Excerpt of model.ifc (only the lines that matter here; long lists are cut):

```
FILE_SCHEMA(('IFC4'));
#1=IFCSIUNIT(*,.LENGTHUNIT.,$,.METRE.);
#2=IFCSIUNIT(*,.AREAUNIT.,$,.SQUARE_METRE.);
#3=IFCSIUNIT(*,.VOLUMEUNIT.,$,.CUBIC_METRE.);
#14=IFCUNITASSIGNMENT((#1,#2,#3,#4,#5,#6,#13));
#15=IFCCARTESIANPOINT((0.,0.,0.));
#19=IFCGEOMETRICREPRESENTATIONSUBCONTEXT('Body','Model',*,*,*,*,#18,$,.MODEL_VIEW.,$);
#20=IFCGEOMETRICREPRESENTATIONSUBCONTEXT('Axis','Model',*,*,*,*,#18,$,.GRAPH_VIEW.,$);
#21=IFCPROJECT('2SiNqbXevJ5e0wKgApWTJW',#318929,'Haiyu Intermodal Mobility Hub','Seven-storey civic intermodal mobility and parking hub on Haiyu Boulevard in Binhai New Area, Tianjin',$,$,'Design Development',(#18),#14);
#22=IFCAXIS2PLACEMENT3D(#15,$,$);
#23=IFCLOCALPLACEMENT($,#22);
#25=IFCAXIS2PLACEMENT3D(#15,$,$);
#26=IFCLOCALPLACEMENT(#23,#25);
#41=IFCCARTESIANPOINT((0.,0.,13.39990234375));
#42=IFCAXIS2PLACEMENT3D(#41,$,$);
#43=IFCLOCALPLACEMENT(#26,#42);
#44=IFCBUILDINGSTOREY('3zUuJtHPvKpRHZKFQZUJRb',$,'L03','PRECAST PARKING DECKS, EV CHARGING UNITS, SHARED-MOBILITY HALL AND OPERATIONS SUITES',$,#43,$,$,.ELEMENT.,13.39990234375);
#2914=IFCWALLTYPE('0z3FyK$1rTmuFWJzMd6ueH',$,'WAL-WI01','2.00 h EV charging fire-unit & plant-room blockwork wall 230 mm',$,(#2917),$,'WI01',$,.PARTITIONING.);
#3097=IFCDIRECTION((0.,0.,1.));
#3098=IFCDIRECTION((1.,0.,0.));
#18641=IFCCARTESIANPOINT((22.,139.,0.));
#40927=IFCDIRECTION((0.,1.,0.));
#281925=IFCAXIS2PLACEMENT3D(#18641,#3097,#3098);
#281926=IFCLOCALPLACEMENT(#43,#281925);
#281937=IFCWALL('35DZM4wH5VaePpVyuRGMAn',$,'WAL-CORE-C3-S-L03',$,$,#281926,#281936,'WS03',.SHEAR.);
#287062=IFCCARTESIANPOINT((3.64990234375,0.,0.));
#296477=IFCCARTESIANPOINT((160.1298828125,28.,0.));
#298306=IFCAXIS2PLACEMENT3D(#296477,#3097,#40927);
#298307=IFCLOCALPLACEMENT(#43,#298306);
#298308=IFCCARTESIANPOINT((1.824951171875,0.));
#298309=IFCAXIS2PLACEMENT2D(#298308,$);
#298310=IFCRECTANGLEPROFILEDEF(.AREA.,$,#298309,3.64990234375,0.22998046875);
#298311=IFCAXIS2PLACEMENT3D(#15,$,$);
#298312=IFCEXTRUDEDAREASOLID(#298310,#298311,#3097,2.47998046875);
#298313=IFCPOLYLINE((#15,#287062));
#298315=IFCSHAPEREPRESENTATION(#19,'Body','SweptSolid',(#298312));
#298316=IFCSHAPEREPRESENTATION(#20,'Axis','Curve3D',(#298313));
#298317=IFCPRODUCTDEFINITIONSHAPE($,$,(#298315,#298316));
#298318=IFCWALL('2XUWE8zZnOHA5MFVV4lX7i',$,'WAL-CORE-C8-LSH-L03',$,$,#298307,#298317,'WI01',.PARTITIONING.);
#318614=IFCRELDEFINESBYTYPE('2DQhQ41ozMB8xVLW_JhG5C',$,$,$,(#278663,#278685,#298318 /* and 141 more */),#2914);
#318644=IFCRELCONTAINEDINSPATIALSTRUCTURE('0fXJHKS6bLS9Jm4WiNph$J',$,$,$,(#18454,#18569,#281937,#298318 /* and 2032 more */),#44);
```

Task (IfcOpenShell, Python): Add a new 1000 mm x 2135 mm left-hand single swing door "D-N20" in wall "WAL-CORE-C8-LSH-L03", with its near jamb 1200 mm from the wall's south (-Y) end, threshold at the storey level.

```python
import numpy as np
import ifcopenshell
import ifcopenshell.api.feature
import ifcopenshell.api.geometry
import ifcopenshell.api.root
import ifcopenshell.api.spatial
import ifcopenshell.geom
import ifcopenshell.util.element
import ifcopenshell.util.placement
import ifcopenshell.util.representation
import ifcopenshell.util.shape
import ifcopenshell.util.unit

model = ifcopenshell.open("model.ifc")
unit_scale = ifcopenshell.util.unit.calculate_unit_scale(model)
settings = ifcopenshell.geom.settings()


def volume(element):
    """Net volume in cubic metres, openings subtracted."""
    shape = ifcopenshell.geom.create_shape(settings, element)
    return ifcopenshell.util.shape.get_volume(shape.geometry)


wall = model.by_id(298318)
storey = ifcopenshell.util.element.get_container(wall, ifc_class="IfcBuildingStorey")
context = ifcopenshell.util.representation.get_context(model, "Model", "Body", "MODEL_VIEW")
before = volume(wall)

width, height, from_end, sill = 1, 2.135, 1.2, 0.0  # metres

# The wall runs along its own X axis, and the end named is its -X end.
wall_shape = ifcopenshell.geom.create_shape(settings, wall)
x, y, z = ifcopenshell.util.shape.get_vertices(wall_shape.geometry).T
start = x.min() + from_end
face, thickness = float(y.min()), float(y.max() - y.min())
wall_matrix = ifcopenshell.util.placement.get_local_placement(wall.ObjectPlacement)
level = ifcopenshell.util.placement.get_local_placement(storey.ObjectPlacement)[2, 3]


def in_wall(x, y):
    """Placement at x, y metres in the wall's axes, at sill height."""
    matrix = wall_matrix.copy()
    matrix[:, 3] = wall_matrix @ np.array([x / unit_scale, y / unit_scale, 0.0, 1.0])
    matrix[2, 3] = level + sill / unit_scale
    return matrix


# Opening: a box that overshoots both wall faces by 50 mm.
opening = ifcopenshell.api.root.create_entity(model, ifc_class="IfcOpeningElement", predefined_type="OPENING")
box = ifcopenshell.api.geometry.add_wall_representation(
    model, context=context, length=width, height=height, thickness=thickness + 0.1
)
ifcopenshell.api.geometry.assign_representation(model, product=opening, representation=box)
ifcopenshell.api.geometry.edit_object_placement(model, product=opening, matrix=in_wall(start, face - 0.05), is_si=False)
ifcopenshell.api.feature.add_feature(model, feature=opening, element=wall)

door = ifcopenshell.api.root.create_entity(model, ifc_class="IfcDoor", name="D-N20", predefined_type="DOOR")
door.OverallWidth, door.OverallHeight = width / unit_scale, height / unit_scale
door.OperationType = "SINGLE_SWING_LEFT"
body = ifcopenshell.api.geometry.add_door_representation(
    model,
    context=context,
    overall_width=door.OverallWidth,
    overall_height=door.OverallHeight,
    operation_type="SINGLE_SWING_LEFT",
    lining_properties={"LiningDepth": thickness / unit_scale, "ThresholdDepth": thickness / unit_scale},
)
ifcopenshell.api.geometry.assign_representation(model, product=door, representation=body)
ifcopenshell.api.spatial.assign_container(model, products=[door], relating_structure=storey)
ifcopenshell.api.feature.add_filling(model, opening=opening, element=door)

# The lining spans the wall, so the door starts at the wall face.
ifcopenshell.api.geometry.edit_object_placement(model, product=door, matrix=in_wall(start, face), is_si=False)

after = volume(wall)

print(f"wall volume {before:.3f} -> {after:.3f} m3")

model.write("model-out.ifc")
```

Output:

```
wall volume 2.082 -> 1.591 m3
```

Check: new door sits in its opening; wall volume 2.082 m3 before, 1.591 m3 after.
